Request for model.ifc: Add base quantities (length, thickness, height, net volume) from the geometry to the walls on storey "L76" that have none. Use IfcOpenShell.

First a look at what the model holds.

```python
import ifcopenshell
import ifcopenshell.util.element
import ifcopenshell.util.unit

model = ifcopenshell.open("model.ifc")
print(model.schema)
for unit_type in ("LENGTHUNIT", "AREAUNIT", "VOLUMEUNIT"):
    print(unit_type, ifcopenshell.util.unit.calculate_unit_scale(model, unit_type))
storey = next(s for s in model.by_type("IfcBuildingStorey") if s.Name == "L76")
walls = [e for e in ifcopenshell.util.element.get_decomposition(storey) if e.is_a("IfcWall")]
for e in sorted(walls, key=lambda e: e.id()):
    print(e.id(), e.is_a(), e.Name, list(ifcopenshell.util.element.get_psets(e, qtos_only=True)), sep=" | ")
```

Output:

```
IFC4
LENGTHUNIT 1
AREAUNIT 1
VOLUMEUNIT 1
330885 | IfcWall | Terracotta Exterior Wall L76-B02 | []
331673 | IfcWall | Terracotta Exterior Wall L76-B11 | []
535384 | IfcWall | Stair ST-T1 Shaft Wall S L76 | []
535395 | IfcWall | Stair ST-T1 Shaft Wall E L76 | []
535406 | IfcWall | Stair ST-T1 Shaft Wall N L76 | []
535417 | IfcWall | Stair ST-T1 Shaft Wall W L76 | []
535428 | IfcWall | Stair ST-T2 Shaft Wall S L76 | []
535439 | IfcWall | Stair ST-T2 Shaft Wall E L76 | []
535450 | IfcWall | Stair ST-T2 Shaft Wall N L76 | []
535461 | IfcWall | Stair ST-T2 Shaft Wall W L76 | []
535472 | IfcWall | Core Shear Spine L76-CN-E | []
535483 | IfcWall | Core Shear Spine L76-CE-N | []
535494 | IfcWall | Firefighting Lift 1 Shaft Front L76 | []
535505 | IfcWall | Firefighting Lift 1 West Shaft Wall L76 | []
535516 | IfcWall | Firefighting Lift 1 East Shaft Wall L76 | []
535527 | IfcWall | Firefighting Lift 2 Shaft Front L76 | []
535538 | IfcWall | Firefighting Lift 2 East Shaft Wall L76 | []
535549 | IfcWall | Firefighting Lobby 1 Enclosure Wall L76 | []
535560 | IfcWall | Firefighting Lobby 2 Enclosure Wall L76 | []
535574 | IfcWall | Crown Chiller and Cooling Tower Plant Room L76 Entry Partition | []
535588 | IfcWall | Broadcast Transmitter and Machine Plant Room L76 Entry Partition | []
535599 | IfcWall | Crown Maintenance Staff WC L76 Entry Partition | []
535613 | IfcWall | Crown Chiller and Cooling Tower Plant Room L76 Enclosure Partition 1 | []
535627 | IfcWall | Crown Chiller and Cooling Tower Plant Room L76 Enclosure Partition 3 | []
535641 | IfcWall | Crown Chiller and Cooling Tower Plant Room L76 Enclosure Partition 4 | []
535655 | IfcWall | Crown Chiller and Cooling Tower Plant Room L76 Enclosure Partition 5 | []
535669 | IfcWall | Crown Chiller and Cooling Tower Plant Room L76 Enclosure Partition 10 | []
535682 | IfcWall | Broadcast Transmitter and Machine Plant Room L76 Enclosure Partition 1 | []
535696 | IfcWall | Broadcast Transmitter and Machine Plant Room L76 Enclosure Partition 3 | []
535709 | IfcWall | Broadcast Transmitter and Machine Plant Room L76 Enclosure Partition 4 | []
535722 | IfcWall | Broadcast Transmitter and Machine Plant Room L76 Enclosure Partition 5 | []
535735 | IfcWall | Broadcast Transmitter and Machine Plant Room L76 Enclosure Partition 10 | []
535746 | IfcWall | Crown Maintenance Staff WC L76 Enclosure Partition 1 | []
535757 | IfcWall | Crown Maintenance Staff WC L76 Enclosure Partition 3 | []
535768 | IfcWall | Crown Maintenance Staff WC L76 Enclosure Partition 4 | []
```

```python
import ifcopenshell
import ifcopenshell.api.pset
import ifcopenshell.geom
import ifcopenshell.util.element
import ifcopenshell.util.shape
import ifcopenshell.util.unit

model = ifcopenshell.open("model.ifc")
unit_scale = ifcopenshell.util.unit.calculate_unit_scale(model)
volume_scale = ifcopenshell.util.unit.calculate_unit_scale(model, "VOLUMEUNIT")
settings = ifcopenshell.geom.settings()

storey = next(s for s in model.by_type("IfcBuildingStorey") if s.Name == "L76")
walls = [e for e in ifcopenshell.util.element.get_decomposition(storey) if e.is_a("IfcWall")]

for e in sorted(walls, key=lambda e: e.id()):
    if ifcopenshell.util.element.get_psets(e, qtos_only=True, should_inherit=False):
        continue
    # Geometry comes back in metres, in the element's own axes.
    shape = ifcopenshell.geom.create_shape(settings, e)
    values = {
        "Length": ifcopenshell.util.shape.get_x(shape.geometry) / unit_scale,
        "Width": ifcopenshell.util.shape.get_y(shape.geometry) / unit_scale,
        "Height": ifcopenshell.util.shape.get_z(shape.geometry) / unit_scale,
        "NetVolume": ifcopenshell.util.shape.get_volume(shape.geometry) / volume_scale,
    }
    qto = ifcopenshell.api.pset.add_qto(model, product=e, name="Qto_WallBaseQuantities")
    ifcopenshell.api.pset.edit_qto(model, qto=qto, properties=values)
    print(e.id(), {k: round(v, 3) for k, v in values.items()})

model.write("model_edited.ifc")
```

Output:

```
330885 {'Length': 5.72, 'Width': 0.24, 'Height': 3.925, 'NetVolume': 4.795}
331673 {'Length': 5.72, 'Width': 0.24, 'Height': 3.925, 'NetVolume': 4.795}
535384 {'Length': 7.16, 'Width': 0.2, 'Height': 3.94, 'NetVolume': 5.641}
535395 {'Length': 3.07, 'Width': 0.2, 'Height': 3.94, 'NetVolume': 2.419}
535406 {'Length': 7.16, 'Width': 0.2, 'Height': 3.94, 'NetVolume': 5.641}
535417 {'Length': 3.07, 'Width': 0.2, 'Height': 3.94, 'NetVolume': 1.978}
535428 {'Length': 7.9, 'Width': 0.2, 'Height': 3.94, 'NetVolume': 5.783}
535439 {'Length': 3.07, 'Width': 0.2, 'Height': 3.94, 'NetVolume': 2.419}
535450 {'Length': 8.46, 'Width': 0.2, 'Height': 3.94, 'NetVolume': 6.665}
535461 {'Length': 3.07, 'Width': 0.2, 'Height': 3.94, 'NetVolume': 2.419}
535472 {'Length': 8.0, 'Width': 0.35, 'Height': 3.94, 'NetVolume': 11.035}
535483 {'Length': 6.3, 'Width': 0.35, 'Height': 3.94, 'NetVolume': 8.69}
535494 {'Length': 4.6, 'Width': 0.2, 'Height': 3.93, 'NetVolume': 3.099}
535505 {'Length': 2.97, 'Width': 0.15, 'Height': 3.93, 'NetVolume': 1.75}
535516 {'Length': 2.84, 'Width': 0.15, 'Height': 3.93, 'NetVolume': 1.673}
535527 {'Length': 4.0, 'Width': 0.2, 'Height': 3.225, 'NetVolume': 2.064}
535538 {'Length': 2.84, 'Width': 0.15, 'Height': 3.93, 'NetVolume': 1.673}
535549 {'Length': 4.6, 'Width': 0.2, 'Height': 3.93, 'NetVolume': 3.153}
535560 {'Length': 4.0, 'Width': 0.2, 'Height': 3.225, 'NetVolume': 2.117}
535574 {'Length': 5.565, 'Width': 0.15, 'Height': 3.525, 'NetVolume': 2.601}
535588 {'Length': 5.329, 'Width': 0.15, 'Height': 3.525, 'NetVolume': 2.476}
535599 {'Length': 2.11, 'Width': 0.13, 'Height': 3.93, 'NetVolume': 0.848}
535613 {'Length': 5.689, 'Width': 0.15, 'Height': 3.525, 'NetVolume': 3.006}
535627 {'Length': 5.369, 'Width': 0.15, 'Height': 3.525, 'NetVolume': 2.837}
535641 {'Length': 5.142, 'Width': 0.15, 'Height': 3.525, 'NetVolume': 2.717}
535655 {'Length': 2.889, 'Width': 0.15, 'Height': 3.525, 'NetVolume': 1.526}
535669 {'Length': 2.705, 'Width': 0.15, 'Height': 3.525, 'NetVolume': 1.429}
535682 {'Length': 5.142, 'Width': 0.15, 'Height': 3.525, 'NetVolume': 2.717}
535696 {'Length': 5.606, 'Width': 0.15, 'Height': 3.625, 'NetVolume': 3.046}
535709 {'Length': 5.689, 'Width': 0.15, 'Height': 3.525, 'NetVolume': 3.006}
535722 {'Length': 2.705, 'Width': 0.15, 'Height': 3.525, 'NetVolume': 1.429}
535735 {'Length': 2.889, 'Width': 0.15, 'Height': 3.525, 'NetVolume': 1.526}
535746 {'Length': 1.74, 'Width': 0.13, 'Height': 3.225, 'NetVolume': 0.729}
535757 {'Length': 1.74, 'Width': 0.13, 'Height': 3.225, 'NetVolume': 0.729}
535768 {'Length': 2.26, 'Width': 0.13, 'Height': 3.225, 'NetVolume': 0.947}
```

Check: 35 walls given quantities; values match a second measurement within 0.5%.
